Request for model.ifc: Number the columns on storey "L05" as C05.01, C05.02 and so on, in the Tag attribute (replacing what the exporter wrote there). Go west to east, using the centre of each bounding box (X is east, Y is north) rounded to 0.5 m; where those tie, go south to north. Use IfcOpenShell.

First a look at what the model holds.

```python
import ifcopenshell
import ifcopenshell.util.element
import ifcopenshell.util.placement

model = ifcopenshell.open("model.ifc")
print(model.schema)
storey = next(s for s in model.by_type("IfcBuildingStorey") if s.Name == "L05")
columns = [e for e in ifcopenshell.util.element.get_decomposition(storey) if e.is_a("IfcColumn")]
for e in sorted(columns, key=lambda e: e.id()):
    origin = ifcopenshell.util.placement.get_local_placement(e.ObjectPlacement)[:3, 3]
    print(e.id(), e.Tag, e.Name, origin.round(2) + 0.0, sep=" | ")
```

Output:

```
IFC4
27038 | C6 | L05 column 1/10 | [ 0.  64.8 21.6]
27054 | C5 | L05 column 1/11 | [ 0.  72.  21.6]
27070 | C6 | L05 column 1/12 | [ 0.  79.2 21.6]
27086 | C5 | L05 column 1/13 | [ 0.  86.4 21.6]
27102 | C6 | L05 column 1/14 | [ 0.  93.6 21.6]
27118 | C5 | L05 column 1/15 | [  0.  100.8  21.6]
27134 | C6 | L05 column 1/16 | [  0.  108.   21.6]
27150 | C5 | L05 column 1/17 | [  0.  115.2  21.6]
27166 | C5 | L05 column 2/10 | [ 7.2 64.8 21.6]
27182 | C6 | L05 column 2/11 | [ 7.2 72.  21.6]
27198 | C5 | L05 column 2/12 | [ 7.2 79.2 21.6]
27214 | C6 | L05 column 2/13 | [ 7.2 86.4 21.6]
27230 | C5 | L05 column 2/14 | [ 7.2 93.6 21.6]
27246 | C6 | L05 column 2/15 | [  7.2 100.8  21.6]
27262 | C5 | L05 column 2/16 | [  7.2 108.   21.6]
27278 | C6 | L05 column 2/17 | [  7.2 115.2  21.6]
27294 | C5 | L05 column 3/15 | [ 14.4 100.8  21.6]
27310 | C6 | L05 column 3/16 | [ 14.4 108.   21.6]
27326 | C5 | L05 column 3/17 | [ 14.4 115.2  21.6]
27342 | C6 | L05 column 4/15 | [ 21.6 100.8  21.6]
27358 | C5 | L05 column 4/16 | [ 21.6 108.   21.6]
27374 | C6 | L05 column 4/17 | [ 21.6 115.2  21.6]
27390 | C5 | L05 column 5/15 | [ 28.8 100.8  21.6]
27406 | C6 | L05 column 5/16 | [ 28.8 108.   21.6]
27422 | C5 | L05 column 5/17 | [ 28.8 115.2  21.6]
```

```python
import ifcopenshell
import ifcopenshell.geom
import ifcopenshell.util.element
import ifcopenshell.util.shape

model = ifcopenshell.open("model.ifc")
settings = ifcopenshell.geom.settings()
settings.set("use-world-coords", True)


def centre(element):
    shape = ifcopenshell.geom.create_shape(settings, element)
    return ifcopenshell.util.shape.get_bbox_centroid(shape.geometry)


storey = next(s for s in model.by_type("IfcBuildingStorey") if s.Name == "L05")
columns = [e for e in ifcopenshell.util.element.get_decomposition(storey) if e.is_a("IfcColumn")]

# Insertion points can sit at a corner or the storey origin, so sort by the geometry (in metres).
centres = {e: centre(e) for e in columns}
columns.sort(key=lambda e: (round(centres[e][0] / 0.5), centres[e][1]))

for i, e in enumerate(columns, start=1):
    number = f"C05.{i:02d}"
    e.Tag = number
    print(e.id(), number)

model.write("model-out.ifc")
```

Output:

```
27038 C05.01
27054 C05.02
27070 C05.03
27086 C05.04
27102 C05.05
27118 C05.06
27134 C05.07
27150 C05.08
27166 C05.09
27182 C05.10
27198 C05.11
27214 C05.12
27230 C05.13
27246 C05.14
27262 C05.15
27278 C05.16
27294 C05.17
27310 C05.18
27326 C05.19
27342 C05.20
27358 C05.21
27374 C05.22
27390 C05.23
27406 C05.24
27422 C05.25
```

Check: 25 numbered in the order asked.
